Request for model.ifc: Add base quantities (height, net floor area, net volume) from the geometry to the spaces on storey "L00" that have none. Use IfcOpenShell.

First a look at what the model holds.

```python
import ifcopenshell
import ifcopenshell.util.element
import ifcopenshell.util.unit

model = ifcopenshell.open("model.ifc")
print(model.schema)
for unit_type in ("LENGTHUNIT", "AREAUNIT", "VOLUMEUNIT"):
    print(unit_type, ifcopenshell.util.unit.calculate_unit_scale(model, unit_type))
storey = next(s for s in model.by_type("IfcBuildingStorey") if s.Name == "L00")
spaces = [e for e in ifcopenshell.util.element.get_decomposition(storey) if e.is_a("IfcSpace")]
for e in sorted(spaces, key=lambda e: e.id()):
    print(e.id(), e.is_a(), e.Name, list(ifcopenshell.util.element.get_psets(e, qtos_only=True)), sep=" | ")
```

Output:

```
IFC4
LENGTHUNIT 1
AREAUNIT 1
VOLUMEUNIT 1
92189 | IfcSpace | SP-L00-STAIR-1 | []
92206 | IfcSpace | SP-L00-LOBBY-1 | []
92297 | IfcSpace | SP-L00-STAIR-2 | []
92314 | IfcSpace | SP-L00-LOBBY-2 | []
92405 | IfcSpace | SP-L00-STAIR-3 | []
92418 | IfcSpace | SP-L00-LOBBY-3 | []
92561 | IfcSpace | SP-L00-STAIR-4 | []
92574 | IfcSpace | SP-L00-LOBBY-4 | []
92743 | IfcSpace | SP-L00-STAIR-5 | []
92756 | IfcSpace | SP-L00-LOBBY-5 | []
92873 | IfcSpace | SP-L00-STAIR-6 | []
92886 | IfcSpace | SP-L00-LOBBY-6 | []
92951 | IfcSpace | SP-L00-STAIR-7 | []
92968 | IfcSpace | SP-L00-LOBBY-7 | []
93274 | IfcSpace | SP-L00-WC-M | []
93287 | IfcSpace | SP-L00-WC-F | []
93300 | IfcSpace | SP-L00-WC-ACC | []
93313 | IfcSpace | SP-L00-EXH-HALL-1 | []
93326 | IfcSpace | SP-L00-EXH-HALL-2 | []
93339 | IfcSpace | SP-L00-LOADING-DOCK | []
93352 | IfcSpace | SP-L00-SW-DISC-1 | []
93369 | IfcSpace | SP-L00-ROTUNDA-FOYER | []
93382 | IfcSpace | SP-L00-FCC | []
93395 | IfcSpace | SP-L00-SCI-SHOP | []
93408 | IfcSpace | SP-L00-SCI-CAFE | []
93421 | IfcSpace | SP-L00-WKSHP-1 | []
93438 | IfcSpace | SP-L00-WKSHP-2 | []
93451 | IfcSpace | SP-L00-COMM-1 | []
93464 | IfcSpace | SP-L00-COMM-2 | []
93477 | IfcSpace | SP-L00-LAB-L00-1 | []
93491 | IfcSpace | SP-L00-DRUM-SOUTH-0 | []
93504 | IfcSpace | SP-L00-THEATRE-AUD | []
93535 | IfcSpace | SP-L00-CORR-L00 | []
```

```python
import ifcopenshell
import ifcopenshell.api.pset
import ifcopenshell.geom
import ifcopenshell.util.element
import ifcopenshell.util.shape
import ifcopenshell.util.unit

model = ifcopenshell.open("model.ifc")
unit_scale = ifcopenshell.util.unit.calculate_unit_scale(model)
area_scale = ifcopenshell.util.unit.calculate_unit_scale(model, "AREAUNIT")
volume_scale = ifcopenshell.util.unit.calculate_unit_scale(model, "VOLUMEUNIT")
settings = ifcopenshell.geom.settings()

storey = next(s for s in model.by_type("IfcBuildingStorey") if s.Name == "L00")
spaces = [e for e in ifcopenshell.util.element.get_decomposition(storey) if e.is_a("IfcSpace")]

for e in sorted(spaces, key=lambda e: e.id()):
    if ifcopenshell.util.element.get_psets(e, qtos_only=True, should_inherit=False):
        continue
    # Geometry comes back in metres, in the element's own axes.
    shape = ifcopenshell.geom.create_shape(settings, e)
    values = {
        "Height": ifcopenshell.util.shape.get_z(shape.geometry) / unit_scale,
        "NetFloorArea": ifcopenshell.util.shape.get_footprint_area(shape.geometry) / area_scale,
        "NetVolume": ifcopenshell.util.shape.get_volume(shape.geometry) / volume_scale,
    }
    qto = ifcopenshell.api.pset.add_qto(model, product=e, name="Qto_SpaceBaseQuantities")
    ifcopenshell.api.pset.edit_qto(model, qto=qto, properties=values)
    print(e.id(), {k: round(v, 3) for k, v in values.items()})

model.write("model_updated.ifc")
```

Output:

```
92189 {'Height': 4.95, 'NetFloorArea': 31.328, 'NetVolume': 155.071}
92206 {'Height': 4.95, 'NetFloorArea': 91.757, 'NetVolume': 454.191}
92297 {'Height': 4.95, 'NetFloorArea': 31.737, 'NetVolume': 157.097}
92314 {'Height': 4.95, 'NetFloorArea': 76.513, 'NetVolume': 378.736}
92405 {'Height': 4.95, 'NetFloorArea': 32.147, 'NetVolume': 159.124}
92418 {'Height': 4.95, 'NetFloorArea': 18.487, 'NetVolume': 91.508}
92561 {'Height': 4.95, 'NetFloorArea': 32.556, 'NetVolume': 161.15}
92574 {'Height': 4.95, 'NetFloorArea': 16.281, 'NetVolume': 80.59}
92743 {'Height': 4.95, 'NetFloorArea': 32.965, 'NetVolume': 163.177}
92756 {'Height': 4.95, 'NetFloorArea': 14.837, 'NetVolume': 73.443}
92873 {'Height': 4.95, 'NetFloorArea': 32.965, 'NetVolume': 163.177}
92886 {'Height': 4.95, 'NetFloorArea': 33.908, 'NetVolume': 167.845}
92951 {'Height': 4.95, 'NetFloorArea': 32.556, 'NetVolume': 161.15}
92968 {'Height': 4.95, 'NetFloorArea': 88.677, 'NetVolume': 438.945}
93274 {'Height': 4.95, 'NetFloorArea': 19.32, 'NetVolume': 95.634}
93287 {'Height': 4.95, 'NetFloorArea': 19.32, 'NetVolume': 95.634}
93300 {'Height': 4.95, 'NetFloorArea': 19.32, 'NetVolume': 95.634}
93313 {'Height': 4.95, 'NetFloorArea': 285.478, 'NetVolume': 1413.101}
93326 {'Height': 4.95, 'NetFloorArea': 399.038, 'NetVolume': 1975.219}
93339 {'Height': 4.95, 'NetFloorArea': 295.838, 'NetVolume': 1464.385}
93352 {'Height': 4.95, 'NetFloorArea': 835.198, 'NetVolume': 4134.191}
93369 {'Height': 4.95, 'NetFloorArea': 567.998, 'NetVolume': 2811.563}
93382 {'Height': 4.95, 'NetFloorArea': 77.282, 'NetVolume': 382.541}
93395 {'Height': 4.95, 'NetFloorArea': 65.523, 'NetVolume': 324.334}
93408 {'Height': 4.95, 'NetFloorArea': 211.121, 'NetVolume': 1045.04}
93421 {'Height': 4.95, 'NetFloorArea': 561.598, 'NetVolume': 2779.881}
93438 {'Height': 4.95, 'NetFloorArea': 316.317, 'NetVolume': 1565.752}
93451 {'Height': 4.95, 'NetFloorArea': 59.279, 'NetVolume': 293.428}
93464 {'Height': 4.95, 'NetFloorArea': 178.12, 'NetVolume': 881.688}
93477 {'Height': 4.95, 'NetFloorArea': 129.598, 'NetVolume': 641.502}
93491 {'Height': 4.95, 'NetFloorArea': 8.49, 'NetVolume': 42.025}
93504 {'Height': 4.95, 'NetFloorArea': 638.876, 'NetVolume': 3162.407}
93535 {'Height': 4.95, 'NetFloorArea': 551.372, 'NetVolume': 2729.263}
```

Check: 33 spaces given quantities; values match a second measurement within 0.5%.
